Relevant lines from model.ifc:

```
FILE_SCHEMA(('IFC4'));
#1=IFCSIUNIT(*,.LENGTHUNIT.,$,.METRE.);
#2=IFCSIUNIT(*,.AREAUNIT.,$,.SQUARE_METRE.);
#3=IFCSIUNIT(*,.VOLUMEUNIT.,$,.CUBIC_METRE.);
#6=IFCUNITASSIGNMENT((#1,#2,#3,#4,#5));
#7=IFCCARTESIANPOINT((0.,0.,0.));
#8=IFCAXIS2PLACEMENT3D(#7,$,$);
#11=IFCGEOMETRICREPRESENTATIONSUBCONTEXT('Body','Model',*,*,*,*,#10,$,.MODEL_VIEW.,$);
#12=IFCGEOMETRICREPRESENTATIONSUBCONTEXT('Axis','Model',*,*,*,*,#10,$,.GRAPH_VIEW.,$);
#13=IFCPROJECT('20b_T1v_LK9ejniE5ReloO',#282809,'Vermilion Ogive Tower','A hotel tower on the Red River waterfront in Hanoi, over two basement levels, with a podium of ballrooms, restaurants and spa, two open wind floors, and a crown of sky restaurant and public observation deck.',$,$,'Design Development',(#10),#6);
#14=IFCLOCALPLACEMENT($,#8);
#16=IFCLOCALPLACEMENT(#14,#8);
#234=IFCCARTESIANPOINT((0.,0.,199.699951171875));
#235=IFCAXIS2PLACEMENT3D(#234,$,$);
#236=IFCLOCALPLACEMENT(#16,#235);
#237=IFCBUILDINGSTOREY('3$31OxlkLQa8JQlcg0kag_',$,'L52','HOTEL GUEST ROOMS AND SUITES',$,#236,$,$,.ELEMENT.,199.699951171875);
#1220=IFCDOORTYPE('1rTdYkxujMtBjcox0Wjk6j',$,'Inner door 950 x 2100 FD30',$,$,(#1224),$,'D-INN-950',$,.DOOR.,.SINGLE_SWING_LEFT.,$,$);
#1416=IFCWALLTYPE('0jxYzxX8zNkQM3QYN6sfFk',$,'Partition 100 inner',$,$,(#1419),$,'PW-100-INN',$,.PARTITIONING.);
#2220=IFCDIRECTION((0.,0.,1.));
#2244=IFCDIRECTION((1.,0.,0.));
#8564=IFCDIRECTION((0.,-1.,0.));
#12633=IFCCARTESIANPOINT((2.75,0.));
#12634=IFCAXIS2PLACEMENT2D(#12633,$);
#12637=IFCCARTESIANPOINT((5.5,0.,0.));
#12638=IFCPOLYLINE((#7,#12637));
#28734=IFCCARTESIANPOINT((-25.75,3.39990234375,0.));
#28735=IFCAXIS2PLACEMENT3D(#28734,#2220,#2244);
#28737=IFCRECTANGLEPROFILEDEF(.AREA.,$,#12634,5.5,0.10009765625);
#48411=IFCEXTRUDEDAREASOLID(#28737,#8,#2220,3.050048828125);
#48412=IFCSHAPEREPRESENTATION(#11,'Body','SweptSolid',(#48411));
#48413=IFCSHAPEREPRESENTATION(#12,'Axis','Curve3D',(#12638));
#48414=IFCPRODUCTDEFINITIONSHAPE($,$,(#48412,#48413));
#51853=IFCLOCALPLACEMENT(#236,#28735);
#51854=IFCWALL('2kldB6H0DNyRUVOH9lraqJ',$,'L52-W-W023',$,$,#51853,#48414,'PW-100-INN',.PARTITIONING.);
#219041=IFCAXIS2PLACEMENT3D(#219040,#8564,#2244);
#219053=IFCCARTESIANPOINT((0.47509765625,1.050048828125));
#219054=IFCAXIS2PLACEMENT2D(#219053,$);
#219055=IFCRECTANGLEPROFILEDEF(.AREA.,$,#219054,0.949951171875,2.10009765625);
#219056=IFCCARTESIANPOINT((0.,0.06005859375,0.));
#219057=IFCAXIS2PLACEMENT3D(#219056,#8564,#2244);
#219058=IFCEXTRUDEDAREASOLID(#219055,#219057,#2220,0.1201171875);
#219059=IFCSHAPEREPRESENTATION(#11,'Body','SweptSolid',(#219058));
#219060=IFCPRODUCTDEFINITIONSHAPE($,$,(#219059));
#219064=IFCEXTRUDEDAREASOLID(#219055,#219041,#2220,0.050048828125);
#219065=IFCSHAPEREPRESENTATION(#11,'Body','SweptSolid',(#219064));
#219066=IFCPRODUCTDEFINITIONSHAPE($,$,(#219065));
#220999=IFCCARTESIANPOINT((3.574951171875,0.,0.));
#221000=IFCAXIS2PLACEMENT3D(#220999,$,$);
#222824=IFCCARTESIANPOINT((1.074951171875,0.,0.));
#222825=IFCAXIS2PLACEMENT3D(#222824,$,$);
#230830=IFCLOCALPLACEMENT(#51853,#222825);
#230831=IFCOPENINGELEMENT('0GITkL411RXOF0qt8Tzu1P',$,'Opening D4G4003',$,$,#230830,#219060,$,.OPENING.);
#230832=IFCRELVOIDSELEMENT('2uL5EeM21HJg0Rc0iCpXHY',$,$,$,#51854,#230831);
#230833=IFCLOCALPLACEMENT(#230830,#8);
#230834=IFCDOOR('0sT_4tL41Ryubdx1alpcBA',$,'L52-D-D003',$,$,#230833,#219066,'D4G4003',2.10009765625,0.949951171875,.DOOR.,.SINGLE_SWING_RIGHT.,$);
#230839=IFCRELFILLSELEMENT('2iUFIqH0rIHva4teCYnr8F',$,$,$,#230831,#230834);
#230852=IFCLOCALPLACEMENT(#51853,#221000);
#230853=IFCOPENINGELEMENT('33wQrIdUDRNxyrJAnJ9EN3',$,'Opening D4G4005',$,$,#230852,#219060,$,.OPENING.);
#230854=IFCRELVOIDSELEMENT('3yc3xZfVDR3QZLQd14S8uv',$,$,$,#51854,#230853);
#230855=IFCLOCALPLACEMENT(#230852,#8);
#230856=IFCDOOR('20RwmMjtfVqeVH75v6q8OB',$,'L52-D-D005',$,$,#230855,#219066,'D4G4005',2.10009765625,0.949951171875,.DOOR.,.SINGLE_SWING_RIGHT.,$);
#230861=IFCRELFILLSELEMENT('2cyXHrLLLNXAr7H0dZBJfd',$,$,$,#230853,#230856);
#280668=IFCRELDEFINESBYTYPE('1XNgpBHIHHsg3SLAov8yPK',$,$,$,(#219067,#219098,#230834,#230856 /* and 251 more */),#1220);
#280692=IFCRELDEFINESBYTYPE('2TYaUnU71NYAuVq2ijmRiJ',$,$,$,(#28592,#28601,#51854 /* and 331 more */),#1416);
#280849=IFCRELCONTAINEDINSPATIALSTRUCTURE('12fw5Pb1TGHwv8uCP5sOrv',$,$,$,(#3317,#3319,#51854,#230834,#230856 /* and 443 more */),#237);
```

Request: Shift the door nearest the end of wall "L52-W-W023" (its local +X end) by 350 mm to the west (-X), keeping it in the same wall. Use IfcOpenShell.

```python
import ifcopenshell
import ifcopenshell.api.geometry
import ifcopenshell.util.placement
import ifcopenshell.util.unit

model = ifcopenshell.open("model.ifc")
unit_scale = ifcopenshell.util.unit.calculate_unit_scale(model)

door = model.by_guid("20RwmMjtfVqeVH75v6q8OB")
opening = door.FillsVoids[0].RelatingOpeningElement
wall = opening.VoidsElements[0].RelatingBuildingElement

wall_matrix = ifcopenshell.util.placement.get_local_placement(wall.ObjectPlacement)
shift = wall_matrix[:3, 0] * -0.35 / unit_scale
before = ifcopenshell.util.placement.get_local_placement(door.ObjectPlacement)[:3, 3].copy()

# The door is placed relative to its opening, so it follows when the opening moves.
matrix = ifcopenshell.util.placement.get_local_placement(opening.ObjectPlacement)
matrix[:3, 3] += shift
ifcopenshell.api.geometry.edit_object_placement(
    model, product=opening, matrix=matrix, is_si=False, should_transform_children=True
)

after = ifcopenshell.util.placement.get_local_placement(door.ObjectPlacement)[:3, 3]
print("door moved by", (after - before).round(3) + 0.0)

model.write("model_edited.ifc")
```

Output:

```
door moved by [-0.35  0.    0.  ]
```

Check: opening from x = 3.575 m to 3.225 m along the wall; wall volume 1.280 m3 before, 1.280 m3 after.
